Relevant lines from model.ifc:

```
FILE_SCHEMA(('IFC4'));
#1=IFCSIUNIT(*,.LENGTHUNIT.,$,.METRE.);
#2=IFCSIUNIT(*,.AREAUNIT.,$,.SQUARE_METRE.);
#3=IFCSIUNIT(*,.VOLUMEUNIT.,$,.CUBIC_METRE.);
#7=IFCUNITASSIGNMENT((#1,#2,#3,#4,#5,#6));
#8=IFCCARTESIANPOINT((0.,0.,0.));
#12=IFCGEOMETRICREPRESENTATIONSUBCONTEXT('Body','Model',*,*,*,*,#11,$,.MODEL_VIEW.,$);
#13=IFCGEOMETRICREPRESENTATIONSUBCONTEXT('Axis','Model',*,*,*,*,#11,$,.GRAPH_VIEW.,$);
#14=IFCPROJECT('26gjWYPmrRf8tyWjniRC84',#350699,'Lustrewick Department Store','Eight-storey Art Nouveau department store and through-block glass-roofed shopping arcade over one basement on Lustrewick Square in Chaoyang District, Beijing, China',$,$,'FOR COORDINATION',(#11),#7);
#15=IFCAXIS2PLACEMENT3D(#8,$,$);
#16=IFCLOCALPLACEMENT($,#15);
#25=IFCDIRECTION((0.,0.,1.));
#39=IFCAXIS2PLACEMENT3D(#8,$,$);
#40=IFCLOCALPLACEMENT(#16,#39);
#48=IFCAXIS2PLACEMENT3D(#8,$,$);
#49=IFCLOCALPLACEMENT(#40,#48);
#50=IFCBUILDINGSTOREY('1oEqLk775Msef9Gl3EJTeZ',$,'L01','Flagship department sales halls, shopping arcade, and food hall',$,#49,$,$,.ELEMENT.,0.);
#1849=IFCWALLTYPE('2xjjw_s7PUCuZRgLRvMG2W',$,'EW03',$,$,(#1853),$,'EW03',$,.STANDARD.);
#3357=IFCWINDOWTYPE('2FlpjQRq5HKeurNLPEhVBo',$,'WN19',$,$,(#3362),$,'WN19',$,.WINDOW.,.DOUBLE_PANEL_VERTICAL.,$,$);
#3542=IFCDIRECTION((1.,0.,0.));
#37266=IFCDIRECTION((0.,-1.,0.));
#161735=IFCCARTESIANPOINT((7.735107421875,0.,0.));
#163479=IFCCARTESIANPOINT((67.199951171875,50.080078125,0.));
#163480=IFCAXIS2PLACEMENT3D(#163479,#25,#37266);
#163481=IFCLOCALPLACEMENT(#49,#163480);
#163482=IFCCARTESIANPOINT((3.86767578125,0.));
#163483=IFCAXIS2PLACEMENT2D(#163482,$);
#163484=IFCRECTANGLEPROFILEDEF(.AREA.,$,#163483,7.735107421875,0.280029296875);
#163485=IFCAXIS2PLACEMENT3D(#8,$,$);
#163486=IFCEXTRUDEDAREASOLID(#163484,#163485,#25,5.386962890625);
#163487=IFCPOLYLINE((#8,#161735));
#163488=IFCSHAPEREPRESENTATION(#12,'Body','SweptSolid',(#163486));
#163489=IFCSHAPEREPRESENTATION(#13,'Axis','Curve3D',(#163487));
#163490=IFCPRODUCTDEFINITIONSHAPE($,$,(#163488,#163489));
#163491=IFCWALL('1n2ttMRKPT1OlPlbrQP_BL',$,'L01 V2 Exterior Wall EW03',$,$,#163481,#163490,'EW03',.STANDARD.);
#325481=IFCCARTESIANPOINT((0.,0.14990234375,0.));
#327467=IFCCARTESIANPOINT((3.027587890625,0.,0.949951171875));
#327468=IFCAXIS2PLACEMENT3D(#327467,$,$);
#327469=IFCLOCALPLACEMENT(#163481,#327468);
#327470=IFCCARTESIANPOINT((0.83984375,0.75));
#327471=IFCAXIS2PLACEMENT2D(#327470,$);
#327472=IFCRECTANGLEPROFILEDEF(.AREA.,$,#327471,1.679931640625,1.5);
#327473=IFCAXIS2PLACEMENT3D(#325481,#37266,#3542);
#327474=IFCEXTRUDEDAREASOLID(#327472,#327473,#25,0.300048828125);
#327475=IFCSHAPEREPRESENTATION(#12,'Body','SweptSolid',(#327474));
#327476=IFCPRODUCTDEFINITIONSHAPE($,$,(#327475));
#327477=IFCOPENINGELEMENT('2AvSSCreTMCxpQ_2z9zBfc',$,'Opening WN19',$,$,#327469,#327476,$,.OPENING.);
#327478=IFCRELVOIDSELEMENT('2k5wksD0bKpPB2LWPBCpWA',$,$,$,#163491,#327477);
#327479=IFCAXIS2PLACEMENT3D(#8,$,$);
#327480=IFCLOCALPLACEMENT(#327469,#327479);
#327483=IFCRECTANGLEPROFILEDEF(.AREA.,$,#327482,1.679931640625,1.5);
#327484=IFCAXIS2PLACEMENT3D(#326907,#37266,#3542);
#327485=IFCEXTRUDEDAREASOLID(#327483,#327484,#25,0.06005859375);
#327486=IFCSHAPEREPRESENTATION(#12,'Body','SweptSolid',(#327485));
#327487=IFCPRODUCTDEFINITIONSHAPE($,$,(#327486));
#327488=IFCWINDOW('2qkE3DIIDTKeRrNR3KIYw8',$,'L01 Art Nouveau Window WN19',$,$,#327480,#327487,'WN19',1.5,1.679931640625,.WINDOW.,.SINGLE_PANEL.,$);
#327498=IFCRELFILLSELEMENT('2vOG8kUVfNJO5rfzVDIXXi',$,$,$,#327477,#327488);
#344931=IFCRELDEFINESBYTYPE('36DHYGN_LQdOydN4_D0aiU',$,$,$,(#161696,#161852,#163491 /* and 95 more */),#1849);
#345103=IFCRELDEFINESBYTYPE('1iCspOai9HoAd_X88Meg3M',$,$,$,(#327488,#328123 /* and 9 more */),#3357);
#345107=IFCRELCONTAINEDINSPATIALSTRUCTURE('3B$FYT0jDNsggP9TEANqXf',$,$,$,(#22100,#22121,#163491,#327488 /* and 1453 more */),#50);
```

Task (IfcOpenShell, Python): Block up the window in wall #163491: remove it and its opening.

```python
import ifcopenshell
import ifcopenshell.api.feature
import ifcopenshell.api.root
import ifcopenshell.geom
import ifcopenshell.util.shape

model = ifcopenshell.open("model.ifc")
settings = ifcopenshell.geom.settings()


def volume(element):
    """Net volume in cubic metres, openings subtracted."""
    shape = ifcopenshell.geom.create_shape(settings, element)
    return ifcopenshell.util.shape.get_volume(shape.geometry)


window = model.by_id(327488)
opening = window.FillsVoids[0].RelatingOpeningElement
wall = opening.VoidsElements[0].RelatingBuildingElement
before = volume(wall)

ifcopenshell.api.root.remove_product(model, product=window)
ifcopenshell.api.feature.remove_feature(model, feature=opening)

after = volume(wall)

print(f"wall volume {before:.3f} -> {after:.3f} m3")

model.write("model_v2.ifc")
```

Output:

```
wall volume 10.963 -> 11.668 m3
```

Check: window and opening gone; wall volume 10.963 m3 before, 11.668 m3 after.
